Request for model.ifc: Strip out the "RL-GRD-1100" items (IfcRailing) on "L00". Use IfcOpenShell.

First a look at what the model holds.

```python
import ifcopenshell
import ifcopenshell.util.element

model = ifcopenshell.open("model.ifc")
print(model.schema)
storey = next(s for s in model.by_type("IfcBuildingStorey") if s.Name == "L00")
railings = [e for e in ifcopenshell.util.element.get_decomposition(storey) if e.is_a("IfcRailing")]
seen = {}
for e in railings:
    element_type = ifcopenshell.util.element.get_type(e)
    name = element_type.Name if element_type not in (None, e) else None
    seen[name] = seen.get(name, 0) + 1
for name, count in sorted(seen.items(), key=str):
    print(count, "x", name)
```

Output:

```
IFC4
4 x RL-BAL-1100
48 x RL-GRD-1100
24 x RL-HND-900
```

```python
import ifcopenshell
import ifcopenshell.api.root
import ifcopenshell.util.element

model = ifcopenshell.open("model.ifc")

storey = next(s for s in model.by_type("IfcBuildingStorey") if s.Name == "L00")
railings = [e for e in ifcopenshell.util.element.get_decomposition(storey) if e.is_a("IfcRailing")]
targets = [e for e in railings if (t := ifcopenshell.util.element.get_type(e)) not in (None, e) and t.Name == "RL-GRD-1100"]

for e in targets:
    ifcopenshell.api.root.remove_product(model, product=e)
print(len(targets), "removed")

model.write("model_rev.ifc")
```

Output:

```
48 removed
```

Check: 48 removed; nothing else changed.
